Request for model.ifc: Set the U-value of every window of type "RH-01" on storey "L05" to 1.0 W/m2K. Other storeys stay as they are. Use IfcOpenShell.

First a look at what the model holds.

```python
import ifcopenshell
import ifcopenshell.util.element

model = ifcopenshell.open("model.ifc")
print(model.schema)
storey = next(s for s in model.by_type("IfcBuildingStorey") if s.Name == "L05")
windows = [e for e in ifcopenshell.util.element.get_decomposition(storey) if e.is_a("IfcWindow")]
seen = {}
for e in windows:
    element_type = ifcopenshell.util.element.get_type(e)
    key = (element_type.Name if element_type != e and element_type else None, ifcopenshell.util.element.get_pset(e, "Pset_WindowCommon", "ThermalTransmittance"))
    seen[key] = seen.get(key, 0) + 1
for (name, value), count in sorted(seen.items(), key=str):
    print(count, "x", name, "|", value)
```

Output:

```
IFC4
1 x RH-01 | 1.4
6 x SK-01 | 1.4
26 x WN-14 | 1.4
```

```python
import ifcopenshell
import ifcopenshell.api.pset
import ifcopenshell.util.element

model = ifcopenshell.open("model.ifc")

storey = next(s for s in model.by_type("IfcBuildingStorey") if s.Name == "L05")
windows = [e for e in ifcopenshell.util.element.get_decomposition(storey) if e.is_a("IfcWindow")]

count = 0
for e in windows:
    element_type = ifcopenshell.util.element.get_type(e)
    if element_type in (None, e) or element_type.Name != "RH-01":
        continue
    # add_pset returns the element's existing set when there is one.
    pset = ifcopenshell.api.pset.add_pset(model, product=e, name="Pset_WindowCommon")
    ifcopenshell.api.pset.edit_pset(model, pset=pset, properties={"ThermalTransmittance": 1.0})
    count += 1

print(count, "windows updated")

model.write("model_updated.ifc")
```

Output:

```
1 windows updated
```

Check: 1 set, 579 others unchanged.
